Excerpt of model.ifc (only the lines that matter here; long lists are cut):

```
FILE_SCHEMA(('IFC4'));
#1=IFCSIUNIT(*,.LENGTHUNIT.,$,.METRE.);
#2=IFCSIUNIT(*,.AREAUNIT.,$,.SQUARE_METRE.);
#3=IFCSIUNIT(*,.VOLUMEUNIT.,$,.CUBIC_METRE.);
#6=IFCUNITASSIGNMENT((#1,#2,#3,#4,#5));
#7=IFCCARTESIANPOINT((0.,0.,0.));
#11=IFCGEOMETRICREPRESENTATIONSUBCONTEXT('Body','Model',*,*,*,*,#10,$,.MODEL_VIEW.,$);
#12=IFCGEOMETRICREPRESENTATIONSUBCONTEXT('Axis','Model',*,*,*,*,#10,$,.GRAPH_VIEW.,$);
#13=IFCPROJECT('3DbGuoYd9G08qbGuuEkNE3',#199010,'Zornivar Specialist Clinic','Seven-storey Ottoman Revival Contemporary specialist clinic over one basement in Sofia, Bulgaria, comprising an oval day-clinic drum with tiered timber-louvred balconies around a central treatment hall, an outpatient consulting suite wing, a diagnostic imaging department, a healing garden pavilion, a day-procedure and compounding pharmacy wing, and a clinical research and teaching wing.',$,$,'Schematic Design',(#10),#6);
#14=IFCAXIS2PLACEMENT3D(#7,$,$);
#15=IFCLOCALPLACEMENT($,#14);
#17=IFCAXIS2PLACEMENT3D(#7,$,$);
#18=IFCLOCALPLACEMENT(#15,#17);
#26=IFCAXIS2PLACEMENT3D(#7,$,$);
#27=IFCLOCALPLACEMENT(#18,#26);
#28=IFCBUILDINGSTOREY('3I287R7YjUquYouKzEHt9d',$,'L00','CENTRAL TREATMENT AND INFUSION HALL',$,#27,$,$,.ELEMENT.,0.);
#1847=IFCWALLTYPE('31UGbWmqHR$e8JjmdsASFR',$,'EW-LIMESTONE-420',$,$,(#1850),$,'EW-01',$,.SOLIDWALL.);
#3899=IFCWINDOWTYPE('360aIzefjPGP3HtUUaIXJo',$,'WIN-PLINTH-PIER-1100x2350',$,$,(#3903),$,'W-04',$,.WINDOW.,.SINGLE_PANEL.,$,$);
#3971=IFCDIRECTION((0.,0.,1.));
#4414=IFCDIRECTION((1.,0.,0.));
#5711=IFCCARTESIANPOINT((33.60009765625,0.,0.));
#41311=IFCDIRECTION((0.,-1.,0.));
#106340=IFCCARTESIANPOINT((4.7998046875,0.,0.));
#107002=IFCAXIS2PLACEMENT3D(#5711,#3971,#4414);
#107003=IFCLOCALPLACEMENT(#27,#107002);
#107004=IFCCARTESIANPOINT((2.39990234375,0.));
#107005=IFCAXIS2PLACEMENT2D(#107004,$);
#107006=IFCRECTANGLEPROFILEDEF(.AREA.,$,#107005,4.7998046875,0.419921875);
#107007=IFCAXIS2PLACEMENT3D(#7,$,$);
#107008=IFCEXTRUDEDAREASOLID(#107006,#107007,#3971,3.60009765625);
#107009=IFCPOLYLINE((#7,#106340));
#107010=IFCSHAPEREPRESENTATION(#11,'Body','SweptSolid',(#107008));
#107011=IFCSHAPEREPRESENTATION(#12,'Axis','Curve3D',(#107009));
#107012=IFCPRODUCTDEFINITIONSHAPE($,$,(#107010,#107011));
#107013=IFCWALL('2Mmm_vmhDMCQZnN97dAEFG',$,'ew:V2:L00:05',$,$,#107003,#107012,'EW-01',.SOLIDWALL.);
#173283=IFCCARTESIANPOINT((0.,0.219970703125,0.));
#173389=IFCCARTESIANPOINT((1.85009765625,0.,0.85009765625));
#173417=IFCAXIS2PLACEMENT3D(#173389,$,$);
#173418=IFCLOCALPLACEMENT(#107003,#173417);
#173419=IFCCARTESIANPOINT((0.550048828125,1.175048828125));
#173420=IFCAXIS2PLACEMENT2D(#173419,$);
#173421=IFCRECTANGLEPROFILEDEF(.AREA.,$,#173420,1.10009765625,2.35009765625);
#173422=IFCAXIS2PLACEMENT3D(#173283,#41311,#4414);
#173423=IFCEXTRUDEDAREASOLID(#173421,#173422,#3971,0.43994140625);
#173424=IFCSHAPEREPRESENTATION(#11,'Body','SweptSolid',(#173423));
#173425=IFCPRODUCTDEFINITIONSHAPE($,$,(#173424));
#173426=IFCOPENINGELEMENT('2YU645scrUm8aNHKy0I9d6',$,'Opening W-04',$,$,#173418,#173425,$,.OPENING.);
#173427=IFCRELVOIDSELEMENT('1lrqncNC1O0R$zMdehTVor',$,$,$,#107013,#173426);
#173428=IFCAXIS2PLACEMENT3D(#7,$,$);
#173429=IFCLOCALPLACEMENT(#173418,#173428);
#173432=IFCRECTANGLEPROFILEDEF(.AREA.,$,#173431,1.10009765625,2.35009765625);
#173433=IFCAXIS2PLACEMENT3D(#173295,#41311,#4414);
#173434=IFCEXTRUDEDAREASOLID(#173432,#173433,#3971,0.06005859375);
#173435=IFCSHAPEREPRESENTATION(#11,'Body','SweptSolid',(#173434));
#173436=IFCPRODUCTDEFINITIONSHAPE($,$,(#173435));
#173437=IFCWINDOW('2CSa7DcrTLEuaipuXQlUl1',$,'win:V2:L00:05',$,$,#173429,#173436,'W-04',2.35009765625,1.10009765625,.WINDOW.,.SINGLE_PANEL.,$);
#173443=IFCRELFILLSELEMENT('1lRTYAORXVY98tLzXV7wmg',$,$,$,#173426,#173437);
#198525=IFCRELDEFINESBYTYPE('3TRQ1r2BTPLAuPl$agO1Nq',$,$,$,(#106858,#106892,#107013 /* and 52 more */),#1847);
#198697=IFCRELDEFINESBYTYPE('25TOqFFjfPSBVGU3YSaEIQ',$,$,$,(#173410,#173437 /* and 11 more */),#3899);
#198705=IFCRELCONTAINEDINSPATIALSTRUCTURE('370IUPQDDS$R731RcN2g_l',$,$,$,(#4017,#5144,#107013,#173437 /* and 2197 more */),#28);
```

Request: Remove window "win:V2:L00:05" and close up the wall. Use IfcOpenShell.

```python
import ifcopenshell
import ifcopenshell.api.feature
import ifcopenshell.api.root
import ifcopenshell.geom
import ifcopenshell.util.shape

model = ifcopenshell.open("model.ifc")
settings = ifcopenshell.geom.settings()


def volume(element):
    """Net volume in cubic metres, openings subtracted."""
    shape = ifcopenshell.geom.create_shape(settings, element)
    return ifcopenshell.util.shape.get_volume(shape.geometry)


window = model.by_guid("2CSa7DcrTLEuaipuXQlUl1")
opening = window.FillsVoids[0].RelatingOpeningElement
wall = opening.VoidsElements[0].RelatingBuildingElement
before = volume(wall)

ifcopenshell.api.root.remove_product(model, product=window)
ifcopenshell.api.feature.remove_feature(model, feature=opening)

after = volume(wall)

print(f"wall volume {before:.3f} -> {after:.3f} m3")

model.write("model_v2.ifc")
```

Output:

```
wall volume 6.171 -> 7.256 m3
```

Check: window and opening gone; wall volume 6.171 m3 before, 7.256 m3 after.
